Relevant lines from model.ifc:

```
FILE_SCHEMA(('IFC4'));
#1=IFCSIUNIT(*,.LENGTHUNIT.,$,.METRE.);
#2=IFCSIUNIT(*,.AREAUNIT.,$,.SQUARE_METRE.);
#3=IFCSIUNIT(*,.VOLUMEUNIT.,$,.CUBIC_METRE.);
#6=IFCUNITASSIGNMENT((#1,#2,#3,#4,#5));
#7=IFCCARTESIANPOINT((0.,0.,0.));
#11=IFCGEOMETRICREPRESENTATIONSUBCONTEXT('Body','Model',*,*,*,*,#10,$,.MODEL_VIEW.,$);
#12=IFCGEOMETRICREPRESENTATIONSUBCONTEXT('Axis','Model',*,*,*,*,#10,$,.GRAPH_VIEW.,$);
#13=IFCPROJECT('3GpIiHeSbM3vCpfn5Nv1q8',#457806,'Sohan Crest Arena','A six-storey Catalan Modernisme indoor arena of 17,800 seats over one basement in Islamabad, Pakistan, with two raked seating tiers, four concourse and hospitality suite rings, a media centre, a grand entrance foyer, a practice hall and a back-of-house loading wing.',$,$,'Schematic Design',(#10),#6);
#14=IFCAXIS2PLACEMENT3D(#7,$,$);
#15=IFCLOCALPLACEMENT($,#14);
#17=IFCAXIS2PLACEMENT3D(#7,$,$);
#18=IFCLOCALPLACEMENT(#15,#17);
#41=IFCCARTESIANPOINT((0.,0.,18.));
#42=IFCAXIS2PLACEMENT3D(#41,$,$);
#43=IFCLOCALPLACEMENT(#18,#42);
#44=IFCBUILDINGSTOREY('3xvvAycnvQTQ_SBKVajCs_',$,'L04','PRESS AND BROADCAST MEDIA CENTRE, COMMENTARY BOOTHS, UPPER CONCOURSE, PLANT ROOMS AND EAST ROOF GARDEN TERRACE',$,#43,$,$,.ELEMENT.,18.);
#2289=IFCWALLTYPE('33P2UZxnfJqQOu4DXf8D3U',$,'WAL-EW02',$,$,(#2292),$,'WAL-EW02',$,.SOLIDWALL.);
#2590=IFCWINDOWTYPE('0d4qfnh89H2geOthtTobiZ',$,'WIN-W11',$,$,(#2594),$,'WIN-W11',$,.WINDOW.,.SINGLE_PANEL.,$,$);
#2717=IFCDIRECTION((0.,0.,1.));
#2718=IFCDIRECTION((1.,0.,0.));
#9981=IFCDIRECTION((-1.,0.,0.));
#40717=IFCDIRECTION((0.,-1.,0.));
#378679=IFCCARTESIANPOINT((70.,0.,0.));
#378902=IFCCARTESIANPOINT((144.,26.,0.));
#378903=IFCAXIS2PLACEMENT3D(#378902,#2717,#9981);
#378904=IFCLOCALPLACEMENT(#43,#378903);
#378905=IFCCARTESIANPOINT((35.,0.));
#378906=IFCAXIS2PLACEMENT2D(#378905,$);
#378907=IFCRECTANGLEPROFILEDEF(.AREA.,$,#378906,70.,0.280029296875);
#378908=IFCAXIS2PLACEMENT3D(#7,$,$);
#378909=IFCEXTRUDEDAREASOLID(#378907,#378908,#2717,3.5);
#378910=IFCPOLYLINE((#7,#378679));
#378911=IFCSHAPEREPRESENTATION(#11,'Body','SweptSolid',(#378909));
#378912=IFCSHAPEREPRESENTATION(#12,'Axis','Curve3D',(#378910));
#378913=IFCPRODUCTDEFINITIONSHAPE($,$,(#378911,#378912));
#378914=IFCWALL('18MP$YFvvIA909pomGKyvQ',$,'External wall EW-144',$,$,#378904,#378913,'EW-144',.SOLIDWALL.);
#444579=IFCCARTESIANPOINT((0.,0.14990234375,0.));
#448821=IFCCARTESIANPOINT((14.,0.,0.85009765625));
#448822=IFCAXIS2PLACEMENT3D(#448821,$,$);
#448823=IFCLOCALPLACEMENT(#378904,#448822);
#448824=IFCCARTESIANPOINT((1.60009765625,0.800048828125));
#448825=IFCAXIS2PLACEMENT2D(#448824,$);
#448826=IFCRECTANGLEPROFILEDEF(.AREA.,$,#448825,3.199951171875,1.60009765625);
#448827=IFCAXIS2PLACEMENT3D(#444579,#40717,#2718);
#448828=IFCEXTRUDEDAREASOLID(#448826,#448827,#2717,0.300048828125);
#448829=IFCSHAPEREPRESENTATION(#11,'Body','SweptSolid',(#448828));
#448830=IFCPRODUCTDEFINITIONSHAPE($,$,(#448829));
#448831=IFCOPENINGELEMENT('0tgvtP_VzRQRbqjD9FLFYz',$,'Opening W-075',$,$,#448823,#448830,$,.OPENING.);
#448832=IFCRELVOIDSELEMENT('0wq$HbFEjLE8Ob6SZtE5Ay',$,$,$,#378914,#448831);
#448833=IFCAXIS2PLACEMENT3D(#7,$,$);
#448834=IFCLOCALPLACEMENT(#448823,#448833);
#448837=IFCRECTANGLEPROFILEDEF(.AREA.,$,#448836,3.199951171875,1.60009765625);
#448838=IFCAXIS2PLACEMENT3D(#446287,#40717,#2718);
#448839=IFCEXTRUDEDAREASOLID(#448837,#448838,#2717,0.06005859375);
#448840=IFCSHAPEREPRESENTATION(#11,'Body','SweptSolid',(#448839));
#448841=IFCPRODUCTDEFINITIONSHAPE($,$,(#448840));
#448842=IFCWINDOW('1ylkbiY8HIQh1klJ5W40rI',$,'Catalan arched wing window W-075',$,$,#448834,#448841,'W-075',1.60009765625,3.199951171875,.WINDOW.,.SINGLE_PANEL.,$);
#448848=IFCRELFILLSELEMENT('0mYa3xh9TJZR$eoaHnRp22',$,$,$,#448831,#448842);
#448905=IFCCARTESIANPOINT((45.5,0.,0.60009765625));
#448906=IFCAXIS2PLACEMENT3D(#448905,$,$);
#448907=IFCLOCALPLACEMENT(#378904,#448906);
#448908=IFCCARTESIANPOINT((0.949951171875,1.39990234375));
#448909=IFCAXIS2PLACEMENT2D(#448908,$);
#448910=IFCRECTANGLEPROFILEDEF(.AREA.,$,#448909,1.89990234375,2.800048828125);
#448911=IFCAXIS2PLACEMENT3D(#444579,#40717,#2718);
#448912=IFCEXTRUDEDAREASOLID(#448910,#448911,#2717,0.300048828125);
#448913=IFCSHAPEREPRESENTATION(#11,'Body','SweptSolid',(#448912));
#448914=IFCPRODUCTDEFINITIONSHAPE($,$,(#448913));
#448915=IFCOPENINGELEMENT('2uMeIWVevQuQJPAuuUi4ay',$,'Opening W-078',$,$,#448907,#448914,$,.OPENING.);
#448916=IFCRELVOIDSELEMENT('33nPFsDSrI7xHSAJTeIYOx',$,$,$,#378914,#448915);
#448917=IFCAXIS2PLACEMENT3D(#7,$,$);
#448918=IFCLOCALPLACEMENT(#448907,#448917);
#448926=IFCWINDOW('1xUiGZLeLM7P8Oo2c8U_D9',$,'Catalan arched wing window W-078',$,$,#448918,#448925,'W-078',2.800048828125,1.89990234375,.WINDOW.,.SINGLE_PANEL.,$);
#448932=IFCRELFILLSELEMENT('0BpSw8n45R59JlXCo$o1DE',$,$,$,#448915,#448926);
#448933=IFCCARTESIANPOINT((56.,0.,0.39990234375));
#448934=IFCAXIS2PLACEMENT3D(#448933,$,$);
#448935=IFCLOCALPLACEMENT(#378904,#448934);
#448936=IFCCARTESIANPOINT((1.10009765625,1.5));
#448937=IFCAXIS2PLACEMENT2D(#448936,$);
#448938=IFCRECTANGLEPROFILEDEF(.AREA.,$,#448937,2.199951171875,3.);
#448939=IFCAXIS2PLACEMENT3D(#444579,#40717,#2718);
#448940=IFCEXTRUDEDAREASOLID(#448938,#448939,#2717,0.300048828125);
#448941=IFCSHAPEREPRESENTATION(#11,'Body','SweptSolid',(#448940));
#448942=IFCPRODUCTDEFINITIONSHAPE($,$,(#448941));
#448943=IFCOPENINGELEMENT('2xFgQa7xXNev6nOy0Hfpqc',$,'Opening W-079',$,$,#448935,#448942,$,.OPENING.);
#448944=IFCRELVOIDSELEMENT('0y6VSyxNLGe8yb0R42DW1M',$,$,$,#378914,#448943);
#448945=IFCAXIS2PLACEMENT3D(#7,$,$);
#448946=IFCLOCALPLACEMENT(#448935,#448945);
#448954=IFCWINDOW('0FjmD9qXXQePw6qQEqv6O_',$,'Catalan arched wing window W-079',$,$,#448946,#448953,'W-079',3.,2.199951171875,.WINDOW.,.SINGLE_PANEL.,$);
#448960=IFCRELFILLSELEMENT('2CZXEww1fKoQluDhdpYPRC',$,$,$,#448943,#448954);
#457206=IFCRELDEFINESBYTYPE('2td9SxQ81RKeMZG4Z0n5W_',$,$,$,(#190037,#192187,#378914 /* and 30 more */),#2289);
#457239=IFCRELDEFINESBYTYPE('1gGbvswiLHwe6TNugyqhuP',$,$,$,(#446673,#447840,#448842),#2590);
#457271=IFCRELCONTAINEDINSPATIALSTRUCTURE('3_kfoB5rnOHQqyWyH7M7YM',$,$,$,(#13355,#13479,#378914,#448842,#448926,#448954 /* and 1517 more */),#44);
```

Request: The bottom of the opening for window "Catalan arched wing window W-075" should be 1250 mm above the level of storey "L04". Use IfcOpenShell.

```python
import numpy as np
import ifcopenshell
import ifcopenshell.api.geometry
import ifcopenshell.geom
import ifcopenshell.util.element
import ifcopenshell.util.placement
import ifcopenshell.util.shape
import ifcopenshell.util.unit

model = ifcopenshell.open("model.ifc")
unit_scale = ifcopenshell.util.unit.calculate_unit_scale(model)

window = model.by_id(448842)
opening = window.FillsVoids[0].RelatingOpeningElement
storey = ifcopenshell.util.element.get_container(window, ifc_class="IfcBuildingStorey")
level = ifcopenshell.util.placement.get_local_placement(storey.ObjectPlacement)[2, 3]

# The opening's origin need not be at the sill, so measure its lowest point.
shape = ifcopenshell.geom.create_shape(ifcopenshell.geom.settings(), opening)
bottom = ifcopenshell.util.shape.get_shape_bottom_elevation(shape, shape.geometry) / unit_scale
dz = level + 1.25 - bottom

shift = np.array([0.0, 0.0, dz])
# The window is placed relative to its opening, so it follows when the opening moves.
matrix = ifcopenshell.util.placement.get_local_placement(opening.ObjectPlacement)
matrix[:3, 3] += shift
ifcopenshell.api.geometry.edit_object_placement(
    model, product=opening, matrix=matrix, is_si=False, should_transform_children=True
)

print(f"moved by {dz * unit_scale:+.3f} m")

model.write("model_updated.ifc")
```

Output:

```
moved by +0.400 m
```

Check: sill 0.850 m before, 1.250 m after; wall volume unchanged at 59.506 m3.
